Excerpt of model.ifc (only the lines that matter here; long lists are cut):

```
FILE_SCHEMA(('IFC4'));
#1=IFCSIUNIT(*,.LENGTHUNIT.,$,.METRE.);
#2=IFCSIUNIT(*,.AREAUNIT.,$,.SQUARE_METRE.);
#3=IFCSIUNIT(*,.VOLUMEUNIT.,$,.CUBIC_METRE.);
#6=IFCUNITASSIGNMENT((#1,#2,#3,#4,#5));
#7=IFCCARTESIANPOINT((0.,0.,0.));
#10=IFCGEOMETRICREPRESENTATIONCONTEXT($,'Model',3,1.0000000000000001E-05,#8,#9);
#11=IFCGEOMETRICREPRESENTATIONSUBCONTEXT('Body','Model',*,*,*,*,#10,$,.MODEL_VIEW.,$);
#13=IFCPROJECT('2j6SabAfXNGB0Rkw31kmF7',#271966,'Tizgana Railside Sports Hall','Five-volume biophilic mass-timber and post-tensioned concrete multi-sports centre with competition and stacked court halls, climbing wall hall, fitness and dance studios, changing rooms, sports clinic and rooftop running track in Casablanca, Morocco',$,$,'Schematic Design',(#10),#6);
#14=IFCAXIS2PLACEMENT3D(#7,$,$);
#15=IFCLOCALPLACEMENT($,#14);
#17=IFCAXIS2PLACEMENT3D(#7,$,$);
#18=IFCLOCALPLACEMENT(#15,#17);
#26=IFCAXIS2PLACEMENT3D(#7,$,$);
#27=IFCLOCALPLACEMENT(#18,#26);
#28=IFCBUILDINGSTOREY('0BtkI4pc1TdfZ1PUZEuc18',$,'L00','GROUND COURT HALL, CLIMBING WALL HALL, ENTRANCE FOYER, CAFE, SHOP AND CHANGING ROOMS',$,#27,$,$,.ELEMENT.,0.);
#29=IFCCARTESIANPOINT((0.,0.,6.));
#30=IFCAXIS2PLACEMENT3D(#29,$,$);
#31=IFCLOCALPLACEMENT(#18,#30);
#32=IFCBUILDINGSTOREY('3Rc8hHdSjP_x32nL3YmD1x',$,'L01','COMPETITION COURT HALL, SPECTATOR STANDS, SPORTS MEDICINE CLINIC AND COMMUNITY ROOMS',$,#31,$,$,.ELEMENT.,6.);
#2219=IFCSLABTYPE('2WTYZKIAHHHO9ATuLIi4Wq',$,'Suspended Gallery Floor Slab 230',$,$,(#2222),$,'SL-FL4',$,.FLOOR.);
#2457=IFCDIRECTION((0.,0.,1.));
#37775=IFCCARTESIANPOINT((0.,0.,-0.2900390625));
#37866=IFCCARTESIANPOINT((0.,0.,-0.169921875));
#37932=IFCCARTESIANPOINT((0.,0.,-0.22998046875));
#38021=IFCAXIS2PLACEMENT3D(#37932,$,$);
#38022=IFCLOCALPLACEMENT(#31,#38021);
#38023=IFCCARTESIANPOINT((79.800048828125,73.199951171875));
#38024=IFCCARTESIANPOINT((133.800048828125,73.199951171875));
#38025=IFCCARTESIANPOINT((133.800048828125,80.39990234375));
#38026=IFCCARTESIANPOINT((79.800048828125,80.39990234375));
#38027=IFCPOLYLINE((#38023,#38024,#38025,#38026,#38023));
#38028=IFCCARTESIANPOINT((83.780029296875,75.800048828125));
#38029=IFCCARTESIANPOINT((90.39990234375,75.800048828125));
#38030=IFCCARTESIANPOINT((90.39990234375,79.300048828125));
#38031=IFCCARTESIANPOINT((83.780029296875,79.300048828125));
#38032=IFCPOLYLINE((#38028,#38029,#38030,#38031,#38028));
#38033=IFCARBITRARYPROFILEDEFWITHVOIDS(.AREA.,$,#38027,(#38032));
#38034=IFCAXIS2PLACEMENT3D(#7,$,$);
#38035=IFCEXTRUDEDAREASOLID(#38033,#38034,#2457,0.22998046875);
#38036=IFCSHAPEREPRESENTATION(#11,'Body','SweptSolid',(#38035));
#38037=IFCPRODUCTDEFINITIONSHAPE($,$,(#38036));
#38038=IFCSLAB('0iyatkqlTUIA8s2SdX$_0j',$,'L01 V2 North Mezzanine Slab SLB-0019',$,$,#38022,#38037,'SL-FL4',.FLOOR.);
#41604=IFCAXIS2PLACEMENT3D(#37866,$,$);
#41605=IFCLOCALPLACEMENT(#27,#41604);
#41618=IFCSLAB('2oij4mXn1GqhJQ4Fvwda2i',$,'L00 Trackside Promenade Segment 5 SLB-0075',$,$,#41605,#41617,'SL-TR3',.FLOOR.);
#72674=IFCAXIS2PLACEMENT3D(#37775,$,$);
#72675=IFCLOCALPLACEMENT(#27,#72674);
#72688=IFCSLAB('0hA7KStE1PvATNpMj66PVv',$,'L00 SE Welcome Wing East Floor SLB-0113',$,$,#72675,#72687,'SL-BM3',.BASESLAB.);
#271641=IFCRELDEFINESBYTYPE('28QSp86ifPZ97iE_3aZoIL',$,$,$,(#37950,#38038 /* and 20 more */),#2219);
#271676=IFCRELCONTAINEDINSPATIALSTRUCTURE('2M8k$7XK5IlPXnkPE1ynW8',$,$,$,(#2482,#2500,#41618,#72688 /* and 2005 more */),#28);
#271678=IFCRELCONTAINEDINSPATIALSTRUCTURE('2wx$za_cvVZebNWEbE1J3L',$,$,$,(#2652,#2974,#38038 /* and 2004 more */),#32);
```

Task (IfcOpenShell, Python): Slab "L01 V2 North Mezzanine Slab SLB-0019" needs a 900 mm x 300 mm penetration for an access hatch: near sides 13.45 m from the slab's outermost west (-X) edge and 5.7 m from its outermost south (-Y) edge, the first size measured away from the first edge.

```python
import numpy as np
import ifcopenshell
import ifcopenshell.api.feature
import ifcopenshell.api.geometry
import ifcopenshell.api.root
import ifcopenshell.geom
import ifcopenshell.util.placement
import ifcopenshell.util.representation
import ifcopenshell.util.shape
import ifcopenshell.util.unit

model = ifcopenshell.open("model.ifc")
unit_scale = ifcopenshell.util.unit.calculate_unit_scale(model)
settings = ifcopenshell.geom.settings()


def volume(element):
    """Net volume in cubic metres, openings subtracted."""
    shape = ifcopenshell.geom.create_shape(settings, element)
    return ifcopenshell.util.shape.get_volume(shape.geometry)


slab = model.by_id(38038)
before = volume(slab)

# Extent in the slab's own axes, in metres. The edges named are its -X and -Y sides.
slab_shape = ifcopenshell.geom.create_shape(settings, slab)
vertices = ifcopenshell.util.shape.get_vertices(slab_shape.geometry)
x_min, y_min, bottom = vertices.min(axis=0)
top = vertices[:, 2].max()

opening = ifcopenshell.api.root.create_entity(model, ifc_class="IfcOpeningElement", name="Access hatch opening", predefined_type="OPENING")
context = ifcopenshell.util.representation.get_context(model, "Model", "Body", "MODEL_VIEW")
width, depth = 0.9, 0.3
outline = [(0.0, 0.0), (width, 0.0), (width, depth), (0.0, depth), (0.0, 0.0)]
# Overshoot both faces by 50 mm so the cut is clean.
shape = ifcopenshell.api.geometry.add_slab_representation(
    model, context=context, depth=top - bottom + 0.1, polyline=outline
)
ifcopenshell.api.geometry.assign_representation(model, product=opening, representation=shape)

matrix = ifcopenshell.util.placement.get_local_placement(slab.ObjectPlacement)
matrix[:, 3] = matrix @ np.append(np.array([x_min + 13.45, y_min + 5.7, bottom - 0.05]) / unit_scale, 1.0)
ifcopenshell.api.geometry.edit_object_placement(model, product=opening, matrix=matrix, is_si=False)
ifcopenshell.api.feature.add_feature(model, feature=opening, element=slab)

after = volume(slab)

print(f"slab volume {before:.3f} -> {after:.3f} m3")

model.write("model_v2.ifc")
```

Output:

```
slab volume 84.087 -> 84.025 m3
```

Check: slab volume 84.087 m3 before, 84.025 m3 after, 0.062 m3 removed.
